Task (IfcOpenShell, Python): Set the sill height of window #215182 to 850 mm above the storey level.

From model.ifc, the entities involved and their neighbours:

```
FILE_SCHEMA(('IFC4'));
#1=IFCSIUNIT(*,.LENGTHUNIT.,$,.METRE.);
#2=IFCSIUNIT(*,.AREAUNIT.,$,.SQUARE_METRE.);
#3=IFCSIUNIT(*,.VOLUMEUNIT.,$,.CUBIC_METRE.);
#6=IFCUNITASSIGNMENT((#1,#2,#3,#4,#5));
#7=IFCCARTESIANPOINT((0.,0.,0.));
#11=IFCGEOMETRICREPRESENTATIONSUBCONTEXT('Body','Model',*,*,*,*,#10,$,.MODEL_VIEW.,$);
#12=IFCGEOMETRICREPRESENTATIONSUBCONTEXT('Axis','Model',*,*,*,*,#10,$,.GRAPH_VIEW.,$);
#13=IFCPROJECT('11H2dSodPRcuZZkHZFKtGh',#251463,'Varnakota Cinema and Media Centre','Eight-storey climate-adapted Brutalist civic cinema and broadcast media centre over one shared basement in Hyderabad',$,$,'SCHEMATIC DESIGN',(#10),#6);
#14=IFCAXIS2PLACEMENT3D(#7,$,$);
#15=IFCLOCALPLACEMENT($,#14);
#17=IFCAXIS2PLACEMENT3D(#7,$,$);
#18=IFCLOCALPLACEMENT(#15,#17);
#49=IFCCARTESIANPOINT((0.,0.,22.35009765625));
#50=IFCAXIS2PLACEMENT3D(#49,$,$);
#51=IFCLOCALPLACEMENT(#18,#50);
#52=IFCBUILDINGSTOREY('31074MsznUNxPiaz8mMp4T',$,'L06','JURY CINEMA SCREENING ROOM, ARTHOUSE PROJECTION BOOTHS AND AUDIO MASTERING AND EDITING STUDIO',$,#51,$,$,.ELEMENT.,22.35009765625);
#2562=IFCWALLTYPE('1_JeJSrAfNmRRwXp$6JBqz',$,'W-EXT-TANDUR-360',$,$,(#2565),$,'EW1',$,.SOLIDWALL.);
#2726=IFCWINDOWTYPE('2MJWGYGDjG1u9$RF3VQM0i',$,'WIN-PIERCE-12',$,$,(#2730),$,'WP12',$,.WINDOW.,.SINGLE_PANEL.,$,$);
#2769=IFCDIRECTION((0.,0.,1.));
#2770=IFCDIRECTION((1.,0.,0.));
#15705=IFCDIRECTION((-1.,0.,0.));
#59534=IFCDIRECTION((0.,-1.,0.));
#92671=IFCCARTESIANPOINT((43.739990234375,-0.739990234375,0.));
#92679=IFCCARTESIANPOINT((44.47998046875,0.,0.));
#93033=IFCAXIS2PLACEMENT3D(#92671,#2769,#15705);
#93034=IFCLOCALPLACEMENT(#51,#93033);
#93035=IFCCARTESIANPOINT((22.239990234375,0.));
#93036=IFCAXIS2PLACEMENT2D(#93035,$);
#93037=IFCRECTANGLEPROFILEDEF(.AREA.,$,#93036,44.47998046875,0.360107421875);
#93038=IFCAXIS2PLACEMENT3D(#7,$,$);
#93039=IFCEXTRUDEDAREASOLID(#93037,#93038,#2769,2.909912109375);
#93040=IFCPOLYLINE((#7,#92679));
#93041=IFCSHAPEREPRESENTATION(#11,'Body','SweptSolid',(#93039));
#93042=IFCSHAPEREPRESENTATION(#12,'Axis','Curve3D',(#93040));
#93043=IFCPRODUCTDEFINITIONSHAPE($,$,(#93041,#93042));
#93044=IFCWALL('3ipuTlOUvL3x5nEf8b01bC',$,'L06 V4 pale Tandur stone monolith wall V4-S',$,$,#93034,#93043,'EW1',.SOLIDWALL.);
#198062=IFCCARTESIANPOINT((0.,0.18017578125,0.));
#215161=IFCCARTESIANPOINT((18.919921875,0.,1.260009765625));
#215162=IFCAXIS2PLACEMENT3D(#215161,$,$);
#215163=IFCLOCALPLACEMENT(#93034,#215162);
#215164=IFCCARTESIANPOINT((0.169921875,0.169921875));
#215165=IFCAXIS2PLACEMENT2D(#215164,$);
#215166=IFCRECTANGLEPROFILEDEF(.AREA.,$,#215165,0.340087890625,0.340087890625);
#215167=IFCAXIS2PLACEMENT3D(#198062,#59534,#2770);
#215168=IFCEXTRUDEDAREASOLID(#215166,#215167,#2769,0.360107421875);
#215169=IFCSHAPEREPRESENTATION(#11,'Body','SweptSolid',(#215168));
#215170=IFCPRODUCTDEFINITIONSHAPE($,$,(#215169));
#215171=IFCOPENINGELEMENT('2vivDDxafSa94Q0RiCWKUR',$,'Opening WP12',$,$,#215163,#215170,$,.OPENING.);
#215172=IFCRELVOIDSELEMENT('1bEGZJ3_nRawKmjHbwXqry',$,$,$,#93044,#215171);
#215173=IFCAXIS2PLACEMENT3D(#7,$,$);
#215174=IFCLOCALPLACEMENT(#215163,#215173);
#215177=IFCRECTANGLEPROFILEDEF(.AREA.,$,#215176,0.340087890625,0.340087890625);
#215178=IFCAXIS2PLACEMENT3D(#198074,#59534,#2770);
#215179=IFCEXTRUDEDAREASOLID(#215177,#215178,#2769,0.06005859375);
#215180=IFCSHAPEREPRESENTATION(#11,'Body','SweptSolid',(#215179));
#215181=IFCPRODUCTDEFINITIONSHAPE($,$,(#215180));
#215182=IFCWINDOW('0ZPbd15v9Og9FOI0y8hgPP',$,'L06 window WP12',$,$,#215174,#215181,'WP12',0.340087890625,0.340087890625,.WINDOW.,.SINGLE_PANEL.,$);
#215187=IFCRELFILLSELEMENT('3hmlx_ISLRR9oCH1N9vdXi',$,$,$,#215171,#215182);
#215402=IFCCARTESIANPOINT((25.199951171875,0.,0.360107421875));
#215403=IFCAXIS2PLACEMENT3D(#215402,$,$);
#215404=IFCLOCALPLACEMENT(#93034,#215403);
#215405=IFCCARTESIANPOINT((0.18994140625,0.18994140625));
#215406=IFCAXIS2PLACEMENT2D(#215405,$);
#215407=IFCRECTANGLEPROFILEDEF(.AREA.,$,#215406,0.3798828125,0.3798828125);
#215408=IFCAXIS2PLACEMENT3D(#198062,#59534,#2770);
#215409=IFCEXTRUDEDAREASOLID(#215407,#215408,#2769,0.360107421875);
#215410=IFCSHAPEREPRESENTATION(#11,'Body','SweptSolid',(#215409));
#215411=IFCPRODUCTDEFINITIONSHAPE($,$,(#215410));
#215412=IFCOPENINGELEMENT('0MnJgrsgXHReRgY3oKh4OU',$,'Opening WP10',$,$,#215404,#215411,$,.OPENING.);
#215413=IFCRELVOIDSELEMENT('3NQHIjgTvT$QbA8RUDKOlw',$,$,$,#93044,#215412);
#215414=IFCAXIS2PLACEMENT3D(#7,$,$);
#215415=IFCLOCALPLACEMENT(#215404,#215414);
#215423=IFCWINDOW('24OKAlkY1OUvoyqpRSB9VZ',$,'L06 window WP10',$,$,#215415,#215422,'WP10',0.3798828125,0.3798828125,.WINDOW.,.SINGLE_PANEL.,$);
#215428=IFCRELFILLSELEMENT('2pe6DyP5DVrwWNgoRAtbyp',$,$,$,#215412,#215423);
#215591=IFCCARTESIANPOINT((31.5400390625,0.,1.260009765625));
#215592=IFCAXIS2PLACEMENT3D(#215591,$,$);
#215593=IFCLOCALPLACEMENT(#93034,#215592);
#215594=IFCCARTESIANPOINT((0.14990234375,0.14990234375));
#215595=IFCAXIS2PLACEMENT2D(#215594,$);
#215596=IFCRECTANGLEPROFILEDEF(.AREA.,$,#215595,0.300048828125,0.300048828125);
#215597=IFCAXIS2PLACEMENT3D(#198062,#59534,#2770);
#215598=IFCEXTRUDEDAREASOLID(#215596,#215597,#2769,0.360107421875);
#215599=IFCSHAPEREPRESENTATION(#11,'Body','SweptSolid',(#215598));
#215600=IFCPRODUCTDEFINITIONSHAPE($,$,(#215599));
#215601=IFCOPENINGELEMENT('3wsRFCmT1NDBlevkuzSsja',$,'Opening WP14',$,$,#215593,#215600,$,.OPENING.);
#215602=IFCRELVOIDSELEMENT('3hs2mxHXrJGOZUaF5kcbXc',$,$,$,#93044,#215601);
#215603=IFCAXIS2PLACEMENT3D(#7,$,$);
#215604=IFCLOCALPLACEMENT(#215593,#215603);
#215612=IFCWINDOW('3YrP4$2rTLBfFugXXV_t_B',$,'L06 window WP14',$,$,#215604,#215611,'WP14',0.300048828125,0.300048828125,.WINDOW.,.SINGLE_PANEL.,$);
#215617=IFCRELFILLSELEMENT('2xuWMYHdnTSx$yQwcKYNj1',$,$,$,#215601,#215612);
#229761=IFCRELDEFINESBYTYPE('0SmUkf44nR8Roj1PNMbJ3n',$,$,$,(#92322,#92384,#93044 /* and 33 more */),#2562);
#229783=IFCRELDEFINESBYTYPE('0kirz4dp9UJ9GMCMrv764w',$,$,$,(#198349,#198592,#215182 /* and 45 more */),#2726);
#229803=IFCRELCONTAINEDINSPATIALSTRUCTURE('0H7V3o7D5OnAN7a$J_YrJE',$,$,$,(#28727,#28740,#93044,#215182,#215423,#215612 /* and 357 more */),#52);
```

```python
import numpy as np
import ifcopenshell
import ifcopenshell.api.geometry
import ifcopenshell.geom
import ifcopenshell.util.element
import ifcopenshell.util.placement
import ifcopenshell.util.shape
import ifcopenshell.util.unit

model = ifcopenshell.open("model.ifc")
unit_scale = ifcopenshell.util.unit.calculate_unit_scale(model)

window = model.by_guid("0ZPbd15v9Og9FOI0y8hgPP")
opening = window.FillsVoids[0].RelatingOpeningElement
storey = ifcopenshell.util.element.get_container(window, ifc_class="IfcBuildingStorey")
level = ifcopenshell.util.placement.get_local_placement(storey.ObjectPlacement)[2, 3]

# The opening's origin need not be at the sill, so measure its lowest point.
shape = ifcopenshell.geom.create_shape(ifcopenshell.geom.settings(), opening)
bottom = ifcopenshell.util.shape.get_shape_bottom_elevation(shape, shape.geometry) / unit_scale
dz = level + 0.85 / unit_scale - bottom

shift = np.array([0.0, 0.0, dz])
# The window is placed relative to its opening, so it follows when the opening moves.
matrix = ifcopenshell.util.placement.get_local_placement(opening.ObjectPlacement)
matrix[:3, 3] += shift
ifcopenshell.api.geometry.edit_object_placement(
    model, product=opening, matrix=matrix, is_si=False, should_transform_children=True
)

print(f"moved by {dz * unit_scale:+.3f} m")

model.write("model_rev.ifc")
```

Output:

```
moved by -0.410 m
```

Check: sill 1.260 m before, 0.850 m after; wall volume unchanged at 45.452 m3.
